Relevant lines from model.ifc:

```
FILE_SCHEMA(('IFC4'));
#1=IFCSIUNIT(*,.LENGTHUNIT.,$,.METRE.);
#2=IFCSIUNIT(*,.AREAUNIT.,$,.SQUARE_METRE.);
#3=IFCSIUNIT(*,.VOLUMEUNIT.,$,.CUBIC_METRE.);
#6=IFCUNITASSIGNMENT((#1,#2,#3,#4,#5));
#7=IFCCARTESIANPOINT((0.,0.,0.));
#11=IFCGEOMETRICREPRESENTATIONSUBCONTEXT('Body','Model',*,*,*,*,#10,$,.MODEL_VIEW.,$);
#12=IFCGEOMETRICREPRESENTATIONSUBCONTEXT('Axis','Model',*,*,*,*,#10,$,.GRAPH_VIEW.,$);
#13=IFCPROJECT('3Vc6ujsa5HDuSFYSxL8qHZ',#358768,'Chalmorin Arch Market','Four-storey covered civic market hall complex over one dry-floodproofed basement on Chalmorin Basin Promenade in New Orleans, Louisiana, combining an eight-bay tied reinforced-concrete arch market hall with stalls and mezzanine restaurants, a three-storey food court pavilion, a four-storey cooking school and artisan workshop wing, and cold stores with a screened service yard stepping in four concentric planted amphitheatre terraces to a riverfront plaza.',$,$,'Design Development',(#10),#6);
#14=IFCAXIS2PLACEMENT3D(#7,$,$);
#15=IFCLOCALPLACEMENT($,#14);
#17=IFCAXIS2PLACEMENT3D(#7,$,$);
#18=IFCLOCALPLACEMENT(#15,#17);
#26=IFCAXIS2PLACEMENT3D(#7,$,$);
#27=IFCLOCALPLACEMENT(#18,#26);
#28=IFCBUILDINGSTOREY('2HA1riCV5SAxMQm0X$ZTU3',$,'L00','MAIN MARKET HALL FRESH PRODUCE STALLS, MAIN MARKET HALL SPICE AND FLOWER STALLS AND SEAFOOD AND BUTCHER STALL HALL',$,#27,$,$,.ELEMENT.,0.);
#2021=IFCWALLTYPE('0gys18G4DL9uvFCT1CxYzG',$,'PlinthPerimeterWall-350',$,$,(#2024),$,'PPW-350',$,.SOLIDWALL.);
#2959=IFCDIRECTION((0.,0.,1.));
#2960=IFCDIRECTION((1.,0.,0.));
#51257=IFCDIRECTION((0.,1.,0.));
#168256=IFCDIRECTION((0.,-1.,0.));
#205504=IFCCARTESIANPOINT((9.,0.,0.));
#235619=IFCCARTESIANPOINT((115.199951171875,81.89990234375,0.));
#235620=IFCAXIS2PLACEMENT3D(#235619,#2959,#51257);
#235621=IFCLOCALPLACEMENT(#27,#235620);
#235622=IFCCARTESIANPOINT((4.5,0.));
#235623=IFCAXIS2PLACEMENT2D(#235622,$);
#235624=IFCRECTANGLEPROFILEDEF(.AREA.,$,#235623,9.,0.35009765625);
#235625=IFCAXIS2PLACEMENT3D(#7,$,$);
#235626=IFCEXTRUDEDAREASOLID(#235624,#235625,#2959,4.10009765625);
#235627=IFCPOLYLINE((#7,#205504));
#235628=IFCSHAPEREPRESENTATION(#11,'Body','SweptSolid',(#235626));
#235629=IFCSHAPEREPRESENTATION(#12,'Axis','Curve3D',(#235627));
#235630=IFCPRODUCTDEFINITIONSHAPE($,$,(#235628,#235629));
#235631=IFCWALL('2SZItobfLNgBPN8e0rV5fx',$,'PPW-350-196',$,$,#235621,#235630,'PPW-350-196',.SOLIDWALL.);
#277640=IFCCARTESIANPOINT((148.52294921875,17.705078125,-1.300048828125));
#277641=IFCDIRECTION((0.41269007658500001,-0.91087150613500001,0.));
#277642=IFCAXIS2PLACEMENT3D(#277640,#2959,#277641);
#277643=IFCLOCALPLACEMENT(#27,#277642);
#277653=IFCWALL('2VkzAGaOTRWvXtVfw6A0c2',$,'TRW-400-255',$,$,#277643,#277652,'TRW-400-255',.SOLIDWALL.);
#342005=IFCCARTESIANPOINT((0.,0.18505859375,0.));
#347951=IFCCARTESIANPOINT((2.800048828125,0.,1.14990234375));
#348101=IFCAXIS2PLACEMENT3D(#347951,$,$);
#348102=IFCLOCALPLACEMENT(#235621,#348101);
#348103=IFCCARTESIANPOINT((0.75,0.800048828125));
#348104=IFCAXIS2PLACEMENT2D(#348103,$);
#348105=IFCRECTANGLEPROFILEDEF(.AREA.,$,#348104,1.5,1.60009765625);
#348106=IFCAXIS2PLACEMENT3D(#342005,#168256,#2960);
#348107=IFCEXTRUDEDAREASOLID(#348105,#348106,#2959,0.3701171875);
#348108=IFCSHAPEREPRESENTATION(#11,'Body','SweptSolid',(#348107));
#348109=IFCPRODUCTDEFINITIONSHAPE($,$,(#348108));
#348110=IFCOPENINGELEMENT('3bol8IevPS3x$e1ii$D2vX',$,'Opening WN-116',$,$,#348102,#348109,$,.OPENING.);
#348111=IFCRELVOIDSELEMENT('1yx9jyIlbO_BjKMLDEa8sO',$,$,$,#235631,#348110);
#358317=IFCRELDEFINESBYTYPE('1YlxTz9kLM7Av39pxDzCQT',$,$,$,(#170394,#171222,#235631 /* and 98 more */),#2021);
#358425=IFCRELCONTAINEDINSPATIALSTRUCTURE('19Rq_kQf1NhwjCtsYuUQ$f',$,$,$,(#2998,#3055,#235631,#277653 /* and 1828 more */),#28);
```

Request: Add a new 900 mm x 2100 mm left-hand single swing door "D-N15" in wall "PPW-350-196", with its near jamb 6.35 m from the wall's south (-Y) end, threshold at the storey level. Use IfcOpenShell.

```python
import numpy as np
import ifcopenshell
import ifcopenshell.api.feature
import ifcopenshell.api.geometry
import ifcopenshell.api.root
import ifcopenshell.api.spatial
import ifcopenshell.geom
import ifcopenshell.util.element
import ifcopenshell.util.placement
import ifcopenshell.util.representation
import ifcopenshell.util.shape
import ifcopenshell.util.unit

model = ifcopenshell.open("model.ifc")
unit_scale = ifcopenshell.util.unit.calculate_unit_scale(model)
settings = ifcopenshell.geom.settings()


def volume(element):
    """Net volume in cubic metres, openings subtracted."""
    shape = ifcopenshell.geom.create_shape(settings, element)
    return ifcopenshell.util.shape.get_volume(shape.geometry)


wall = model.by_guid("2SZItobfLNgBPN8e0rV5fx")
storey = ifcopenshell.util.element.get_container(wall, ifc_class="IfcBuildingStorey")
context = ifcopenshell.util.representation.get_context(model, "Model", "Body", "MODEL_VIEW")
before = volume(wall)

width, height, from_end, sill = 0.9, 2.1, 6.35, 0.0  # metres

# The wall runs along its own X axis, and the end named is its -X end.
wall_shape = ifcopenshell.geom.create_shape(settings, wall)
x, y, z = ifcopenshell.util.shape.get_vertices(wall_shape.geometry).T
start = x.min() + from_end
face, thickness = float(y.min()), float(y.max() - y.min())
wall_matrix = ifcopenshell.util.placement.get_local_placement(wall.ObjectPlacement)
level = ifcopenshell.util.placement.get_local_placement(storey.ObjectPlacement)[2, 3]


def in_wall(x, y):
    """Placement at x, y metres in the wall's axes, at sill height."""
    matrix = wall_matrix.copy()
    matrix[:, 3] = wall_matrix @ np.array([x / unit_scale, y / unit_scale, 0.0, 1.0])
    matrix[2, 3] = level + sill / unit_scale
    return matrix


# Opening: a box that overshoots both wall faces by 50 mm.
opening = ifcopenshell.api.root.create_entity(model, ifc_class="IfcOpeningElement", predefined_type="OPENING")
box = ifcopenshell.api.geometry.add_wall_representation(
    model, context=context, length=width, height=height, thickness=thickness + 0.1
)
ifcopenshell.api.geometry.assign_representation(model, product=opening, representation=box)
ifcopenshell.api.geometry.edit_object_placement(model, product=opening, matrix=in_wall(start, face - 0.05), is_si=False)
ifcopenshell.api.feature.add_feature(model, feature=opening, element=wall)

door = ifcopenshell.api.root.create_entity(model, ifc_class="IfcDoor", name="D-N15", predefined_type="DOOR")
door.OverallWidth, door.OverallHeight = width / unit_scale, height / unit_scale
door.OperationType = "SINGLE_SWING_LEFT"
body = ifcopenshell.api.geometry.add_door_representation(
    model,
    context=context,
    overall_width=door.OverallWidth,
    overall_height=door.OverallHeight,
    operation_type="SINGLE_SWING_LEFT",
    lining_properties={"LiningDepth": thickness / unit_scale, "ThresholdDepth": thickness / unit_scale},
)
ifcopenshell.api.geometry.assign_representation(model, product=door, representation=body)
ifcopenshell.api.spatial.assign_container(model, products=[door], relating_structure=storey)
ifcopenshell.api.feature.add_filling(model, opening=opening, element=door)

# The lining spans the wall, so the door starts at the wall face.
ifcopenshell.api.geometry.edit_object_placement(model, product=door, matrix=in_wall(start, face), is_si=False)

after = volume(wall)

print(f"wall volume {before:.3f} -> {after:.3f} m3")

model.write("model_rev.ifc")
```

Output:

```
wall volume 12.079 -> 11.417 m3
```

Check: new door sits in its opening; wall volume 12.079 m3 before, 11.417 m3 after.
